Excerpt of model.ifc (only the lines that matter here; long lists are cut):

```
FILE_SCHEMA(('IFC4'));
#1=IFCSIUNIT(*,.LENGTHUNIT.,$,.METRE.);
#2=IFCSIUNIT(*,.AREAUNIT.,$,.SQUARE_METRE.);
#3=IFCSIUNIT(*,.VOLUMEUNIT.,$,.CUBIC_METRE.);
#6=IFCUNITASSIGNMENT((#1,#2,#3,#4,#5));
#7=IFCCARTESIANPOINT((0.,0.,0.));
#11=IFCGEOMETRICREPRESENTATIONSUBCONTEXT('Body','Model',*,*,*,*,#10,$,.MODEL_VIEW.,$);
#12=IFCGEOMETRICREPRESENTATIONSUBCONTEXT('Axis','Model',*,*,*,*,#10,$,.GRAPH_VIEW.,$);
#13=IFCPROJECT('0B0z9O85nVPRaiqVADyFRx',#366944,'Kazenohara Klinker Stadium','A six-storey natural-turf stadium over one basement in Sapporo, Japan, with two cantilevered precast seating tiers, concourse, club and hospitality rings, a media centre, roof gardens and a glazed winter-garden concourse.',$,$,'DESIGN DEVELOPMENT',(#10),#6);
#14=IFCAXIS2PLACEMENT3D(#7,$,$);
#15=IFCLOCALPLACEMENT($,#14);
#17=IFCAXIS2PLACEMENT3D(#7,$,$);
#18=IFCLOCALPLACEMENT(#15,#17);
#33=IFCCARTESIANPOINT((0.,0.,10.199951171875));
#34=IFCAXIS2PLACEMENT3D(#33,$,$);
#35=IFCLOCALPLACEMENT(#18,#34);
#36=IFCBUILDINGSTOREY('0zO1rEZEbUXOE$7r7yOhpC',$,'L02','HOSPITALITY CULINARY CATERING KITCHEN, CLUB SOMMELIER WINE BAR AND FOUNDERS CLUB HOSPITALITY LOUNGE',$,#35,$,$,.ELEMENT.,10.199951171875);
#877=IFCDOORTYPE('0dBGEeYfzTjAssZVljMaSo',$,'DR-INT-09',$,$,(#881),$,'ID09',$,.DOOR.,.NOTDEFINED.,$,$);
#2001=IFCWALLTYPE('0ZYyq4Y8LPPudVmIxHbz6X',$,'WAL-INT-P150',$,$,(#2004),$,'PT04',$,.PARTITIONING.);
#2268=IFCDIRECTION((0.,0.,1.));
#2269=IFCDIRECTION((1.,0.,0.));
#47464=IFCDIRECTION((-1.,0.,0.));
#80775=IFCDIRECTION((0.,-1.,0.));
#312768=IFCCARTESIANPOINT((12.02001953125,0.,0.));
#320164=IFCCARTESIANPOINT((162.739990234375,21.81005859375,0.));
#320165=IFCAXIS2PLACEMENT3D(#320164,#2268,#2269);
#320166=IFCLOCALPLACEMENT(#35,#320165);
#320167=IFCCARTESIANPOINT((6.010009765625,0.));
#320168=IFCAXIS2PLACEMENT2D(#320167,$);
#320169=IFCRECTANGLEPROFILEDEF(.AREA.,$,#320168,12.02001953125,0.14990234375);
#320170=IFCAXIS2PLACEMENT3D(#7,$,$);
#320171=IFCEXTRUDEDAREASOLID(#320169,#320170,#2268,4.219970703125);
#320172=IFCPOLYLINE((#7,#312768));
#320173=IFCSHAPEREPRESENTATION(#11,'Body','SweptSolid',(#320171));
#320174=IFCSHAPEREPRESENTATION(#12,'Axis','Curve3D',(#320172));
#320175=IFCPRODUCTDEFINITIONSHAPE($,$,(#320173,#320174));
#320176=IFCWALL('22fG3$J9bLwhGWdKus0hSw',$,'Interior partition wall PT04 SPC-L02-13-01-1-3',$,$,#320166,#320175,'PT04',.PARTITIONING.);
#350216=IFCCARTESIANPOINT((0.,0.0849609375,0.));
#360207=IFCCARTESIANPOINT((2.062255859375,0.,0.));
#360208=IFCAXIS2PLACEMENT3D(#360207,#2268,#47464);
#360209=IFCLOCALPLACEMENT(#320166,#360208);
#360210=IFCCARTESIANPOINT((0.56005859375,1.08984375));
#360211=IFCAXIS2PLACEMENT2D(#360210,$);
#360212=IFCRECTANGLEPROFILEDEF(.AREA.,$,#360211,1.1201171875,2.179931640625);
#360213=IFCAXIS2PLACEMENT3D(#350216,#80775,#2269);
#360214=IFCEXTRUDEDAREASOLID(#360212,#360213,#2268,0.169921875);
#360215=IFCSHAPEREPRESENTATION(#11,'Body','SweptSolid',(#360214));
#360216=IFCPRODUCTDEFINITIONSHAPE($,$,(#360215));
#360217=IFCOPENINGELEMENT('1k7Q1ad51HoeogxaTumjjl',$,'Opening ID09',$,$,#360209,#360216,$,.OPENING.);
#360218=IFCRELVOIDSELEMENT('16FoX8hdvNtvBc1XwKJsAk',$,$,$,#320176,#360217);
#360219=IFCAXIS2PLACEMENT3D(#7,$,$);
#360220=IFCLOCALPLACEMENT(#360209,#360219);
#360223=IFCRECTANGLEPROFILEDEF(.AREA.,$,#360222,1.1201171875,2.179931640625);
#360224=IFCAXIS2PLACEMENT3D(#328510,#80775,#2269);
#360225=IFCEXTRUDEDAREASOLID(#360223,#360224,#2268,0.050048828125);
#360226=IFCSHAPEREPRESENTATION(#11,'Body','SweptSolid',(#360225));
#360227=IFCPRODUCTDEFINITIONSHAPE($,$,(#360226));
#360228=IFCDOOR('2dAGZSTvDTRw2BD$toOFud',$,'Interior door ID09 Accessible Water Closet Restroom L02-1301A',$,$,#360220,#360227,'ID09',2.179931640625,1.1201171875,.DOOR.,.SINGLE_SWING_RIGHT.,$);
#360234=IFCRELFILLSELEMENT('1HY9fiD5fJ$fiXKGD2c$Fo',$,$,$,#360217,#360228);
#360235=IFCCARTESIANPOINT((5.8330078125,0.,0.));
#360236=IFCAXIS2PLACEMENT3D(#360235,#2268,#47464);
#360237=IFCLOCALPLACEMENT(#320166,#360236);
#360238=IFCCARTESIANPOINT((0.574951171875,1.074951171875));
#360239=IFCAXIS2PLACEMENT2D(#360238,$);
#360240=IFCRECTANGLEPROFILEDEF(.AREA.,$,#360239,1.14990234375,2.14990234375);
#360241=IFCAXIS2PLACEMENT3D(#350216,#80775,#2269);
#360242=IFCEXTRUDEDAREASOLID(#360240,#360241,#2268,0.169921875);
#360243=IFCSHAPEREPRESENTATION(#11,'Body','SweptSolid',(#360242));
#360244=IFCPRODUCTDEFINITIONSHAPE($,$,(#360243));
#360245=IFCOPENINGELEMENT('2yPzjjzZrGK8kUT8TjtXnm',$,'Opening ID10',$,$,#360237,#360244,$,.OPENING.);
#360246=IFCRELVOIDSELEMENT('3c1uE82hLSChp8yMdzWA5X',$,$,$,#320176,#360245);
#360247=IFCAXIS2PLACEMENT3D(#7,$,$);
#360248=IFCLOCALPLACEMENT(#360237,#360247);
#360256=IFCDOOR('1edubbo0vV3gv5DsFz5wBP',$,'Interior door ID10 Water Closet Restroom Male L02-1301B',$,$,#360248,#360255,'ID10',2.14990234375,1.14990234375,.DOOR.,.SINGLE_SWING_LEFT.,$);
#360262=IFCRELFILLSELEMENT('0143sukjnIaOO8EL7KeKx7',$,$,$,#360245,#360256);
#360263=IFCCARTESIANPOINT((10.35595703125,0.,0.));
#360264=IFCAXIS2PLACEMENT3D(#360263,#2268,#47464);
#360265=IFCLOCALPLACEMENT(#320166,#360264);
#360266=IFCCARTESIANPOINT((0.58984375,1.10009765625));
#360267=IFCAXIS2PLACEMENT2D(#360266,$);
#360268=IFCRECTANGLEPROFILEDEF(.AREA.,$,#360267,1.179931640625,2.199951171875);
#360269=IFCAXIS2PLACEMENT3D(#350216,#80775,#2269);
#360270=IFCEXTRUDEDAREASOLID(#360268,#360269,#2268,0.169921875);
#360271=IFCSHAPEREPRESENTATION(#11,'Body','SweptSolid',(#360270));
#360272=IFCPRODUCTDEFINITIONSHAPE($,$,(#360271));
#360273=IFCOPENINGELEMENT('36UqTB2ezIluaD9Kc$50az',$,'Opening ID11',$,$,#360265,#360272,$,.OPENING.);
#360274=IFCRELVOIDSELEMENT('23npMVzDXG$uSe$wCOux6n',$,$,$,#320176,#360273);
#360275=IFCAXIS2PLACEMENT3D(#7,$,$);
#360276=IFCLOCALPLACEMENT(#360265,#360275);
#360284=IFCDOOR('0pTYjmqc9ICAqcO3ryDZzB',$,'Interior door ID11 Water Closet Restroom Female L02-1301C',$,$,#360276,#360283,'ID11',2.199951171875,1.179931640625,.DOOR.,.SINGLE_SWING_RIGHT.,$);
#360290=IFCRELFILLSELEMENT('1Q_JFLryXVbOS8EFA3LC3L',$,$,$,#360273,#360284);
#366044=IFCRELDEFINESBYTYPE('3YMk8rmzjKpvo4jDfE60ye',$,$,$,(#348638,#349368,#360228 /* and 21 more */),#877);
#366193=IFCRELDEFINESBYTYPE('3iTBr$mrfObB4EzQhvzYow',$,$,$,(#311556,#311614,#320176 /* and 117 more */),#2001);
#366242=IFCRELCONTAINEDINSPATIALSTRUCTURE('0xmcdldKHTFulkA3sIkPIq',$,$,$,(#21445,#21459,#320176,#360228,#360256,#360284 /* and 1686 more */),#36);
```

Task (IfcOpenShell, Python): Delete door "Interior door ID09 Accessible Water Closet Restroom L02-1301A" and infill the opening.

```python
import ifcopenshell
import ifcopenshell.api.feature
import ifcopenshell.api.root
import ifcopenshell.geom
import ifcopenshell.util.shape

model = ifcopenshell.open("model.ifc")
settings = ifcopenshell.geom.settings()


def volume(element):
    """Net volume in cubic metres, openings subtracted."""
    shape = ifcopenshell.geom.create_shape(settings, element)
    return ifcopenshell.util.shape.get_volume(shape.geometry)


door = model.by_id(360228)
opening = door.FillsVoids[0].RelatingOpeningElement
wall = opening.VoidsElements[0].RelatingBuildingElement
before = volume(wall)

ifcopenshell.api.root.remove_product(model, product=door)
ifcopenshell.api.feature.remove_feature(model, feature=opening)

after = volume(wall)

print(f"wall volume {before:.3f} -> {after:.3f} m3")

model.write("model_updated.ifc")
```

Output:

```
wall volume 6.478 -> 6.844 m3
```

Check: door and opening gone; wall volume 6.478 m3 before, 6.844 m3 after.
